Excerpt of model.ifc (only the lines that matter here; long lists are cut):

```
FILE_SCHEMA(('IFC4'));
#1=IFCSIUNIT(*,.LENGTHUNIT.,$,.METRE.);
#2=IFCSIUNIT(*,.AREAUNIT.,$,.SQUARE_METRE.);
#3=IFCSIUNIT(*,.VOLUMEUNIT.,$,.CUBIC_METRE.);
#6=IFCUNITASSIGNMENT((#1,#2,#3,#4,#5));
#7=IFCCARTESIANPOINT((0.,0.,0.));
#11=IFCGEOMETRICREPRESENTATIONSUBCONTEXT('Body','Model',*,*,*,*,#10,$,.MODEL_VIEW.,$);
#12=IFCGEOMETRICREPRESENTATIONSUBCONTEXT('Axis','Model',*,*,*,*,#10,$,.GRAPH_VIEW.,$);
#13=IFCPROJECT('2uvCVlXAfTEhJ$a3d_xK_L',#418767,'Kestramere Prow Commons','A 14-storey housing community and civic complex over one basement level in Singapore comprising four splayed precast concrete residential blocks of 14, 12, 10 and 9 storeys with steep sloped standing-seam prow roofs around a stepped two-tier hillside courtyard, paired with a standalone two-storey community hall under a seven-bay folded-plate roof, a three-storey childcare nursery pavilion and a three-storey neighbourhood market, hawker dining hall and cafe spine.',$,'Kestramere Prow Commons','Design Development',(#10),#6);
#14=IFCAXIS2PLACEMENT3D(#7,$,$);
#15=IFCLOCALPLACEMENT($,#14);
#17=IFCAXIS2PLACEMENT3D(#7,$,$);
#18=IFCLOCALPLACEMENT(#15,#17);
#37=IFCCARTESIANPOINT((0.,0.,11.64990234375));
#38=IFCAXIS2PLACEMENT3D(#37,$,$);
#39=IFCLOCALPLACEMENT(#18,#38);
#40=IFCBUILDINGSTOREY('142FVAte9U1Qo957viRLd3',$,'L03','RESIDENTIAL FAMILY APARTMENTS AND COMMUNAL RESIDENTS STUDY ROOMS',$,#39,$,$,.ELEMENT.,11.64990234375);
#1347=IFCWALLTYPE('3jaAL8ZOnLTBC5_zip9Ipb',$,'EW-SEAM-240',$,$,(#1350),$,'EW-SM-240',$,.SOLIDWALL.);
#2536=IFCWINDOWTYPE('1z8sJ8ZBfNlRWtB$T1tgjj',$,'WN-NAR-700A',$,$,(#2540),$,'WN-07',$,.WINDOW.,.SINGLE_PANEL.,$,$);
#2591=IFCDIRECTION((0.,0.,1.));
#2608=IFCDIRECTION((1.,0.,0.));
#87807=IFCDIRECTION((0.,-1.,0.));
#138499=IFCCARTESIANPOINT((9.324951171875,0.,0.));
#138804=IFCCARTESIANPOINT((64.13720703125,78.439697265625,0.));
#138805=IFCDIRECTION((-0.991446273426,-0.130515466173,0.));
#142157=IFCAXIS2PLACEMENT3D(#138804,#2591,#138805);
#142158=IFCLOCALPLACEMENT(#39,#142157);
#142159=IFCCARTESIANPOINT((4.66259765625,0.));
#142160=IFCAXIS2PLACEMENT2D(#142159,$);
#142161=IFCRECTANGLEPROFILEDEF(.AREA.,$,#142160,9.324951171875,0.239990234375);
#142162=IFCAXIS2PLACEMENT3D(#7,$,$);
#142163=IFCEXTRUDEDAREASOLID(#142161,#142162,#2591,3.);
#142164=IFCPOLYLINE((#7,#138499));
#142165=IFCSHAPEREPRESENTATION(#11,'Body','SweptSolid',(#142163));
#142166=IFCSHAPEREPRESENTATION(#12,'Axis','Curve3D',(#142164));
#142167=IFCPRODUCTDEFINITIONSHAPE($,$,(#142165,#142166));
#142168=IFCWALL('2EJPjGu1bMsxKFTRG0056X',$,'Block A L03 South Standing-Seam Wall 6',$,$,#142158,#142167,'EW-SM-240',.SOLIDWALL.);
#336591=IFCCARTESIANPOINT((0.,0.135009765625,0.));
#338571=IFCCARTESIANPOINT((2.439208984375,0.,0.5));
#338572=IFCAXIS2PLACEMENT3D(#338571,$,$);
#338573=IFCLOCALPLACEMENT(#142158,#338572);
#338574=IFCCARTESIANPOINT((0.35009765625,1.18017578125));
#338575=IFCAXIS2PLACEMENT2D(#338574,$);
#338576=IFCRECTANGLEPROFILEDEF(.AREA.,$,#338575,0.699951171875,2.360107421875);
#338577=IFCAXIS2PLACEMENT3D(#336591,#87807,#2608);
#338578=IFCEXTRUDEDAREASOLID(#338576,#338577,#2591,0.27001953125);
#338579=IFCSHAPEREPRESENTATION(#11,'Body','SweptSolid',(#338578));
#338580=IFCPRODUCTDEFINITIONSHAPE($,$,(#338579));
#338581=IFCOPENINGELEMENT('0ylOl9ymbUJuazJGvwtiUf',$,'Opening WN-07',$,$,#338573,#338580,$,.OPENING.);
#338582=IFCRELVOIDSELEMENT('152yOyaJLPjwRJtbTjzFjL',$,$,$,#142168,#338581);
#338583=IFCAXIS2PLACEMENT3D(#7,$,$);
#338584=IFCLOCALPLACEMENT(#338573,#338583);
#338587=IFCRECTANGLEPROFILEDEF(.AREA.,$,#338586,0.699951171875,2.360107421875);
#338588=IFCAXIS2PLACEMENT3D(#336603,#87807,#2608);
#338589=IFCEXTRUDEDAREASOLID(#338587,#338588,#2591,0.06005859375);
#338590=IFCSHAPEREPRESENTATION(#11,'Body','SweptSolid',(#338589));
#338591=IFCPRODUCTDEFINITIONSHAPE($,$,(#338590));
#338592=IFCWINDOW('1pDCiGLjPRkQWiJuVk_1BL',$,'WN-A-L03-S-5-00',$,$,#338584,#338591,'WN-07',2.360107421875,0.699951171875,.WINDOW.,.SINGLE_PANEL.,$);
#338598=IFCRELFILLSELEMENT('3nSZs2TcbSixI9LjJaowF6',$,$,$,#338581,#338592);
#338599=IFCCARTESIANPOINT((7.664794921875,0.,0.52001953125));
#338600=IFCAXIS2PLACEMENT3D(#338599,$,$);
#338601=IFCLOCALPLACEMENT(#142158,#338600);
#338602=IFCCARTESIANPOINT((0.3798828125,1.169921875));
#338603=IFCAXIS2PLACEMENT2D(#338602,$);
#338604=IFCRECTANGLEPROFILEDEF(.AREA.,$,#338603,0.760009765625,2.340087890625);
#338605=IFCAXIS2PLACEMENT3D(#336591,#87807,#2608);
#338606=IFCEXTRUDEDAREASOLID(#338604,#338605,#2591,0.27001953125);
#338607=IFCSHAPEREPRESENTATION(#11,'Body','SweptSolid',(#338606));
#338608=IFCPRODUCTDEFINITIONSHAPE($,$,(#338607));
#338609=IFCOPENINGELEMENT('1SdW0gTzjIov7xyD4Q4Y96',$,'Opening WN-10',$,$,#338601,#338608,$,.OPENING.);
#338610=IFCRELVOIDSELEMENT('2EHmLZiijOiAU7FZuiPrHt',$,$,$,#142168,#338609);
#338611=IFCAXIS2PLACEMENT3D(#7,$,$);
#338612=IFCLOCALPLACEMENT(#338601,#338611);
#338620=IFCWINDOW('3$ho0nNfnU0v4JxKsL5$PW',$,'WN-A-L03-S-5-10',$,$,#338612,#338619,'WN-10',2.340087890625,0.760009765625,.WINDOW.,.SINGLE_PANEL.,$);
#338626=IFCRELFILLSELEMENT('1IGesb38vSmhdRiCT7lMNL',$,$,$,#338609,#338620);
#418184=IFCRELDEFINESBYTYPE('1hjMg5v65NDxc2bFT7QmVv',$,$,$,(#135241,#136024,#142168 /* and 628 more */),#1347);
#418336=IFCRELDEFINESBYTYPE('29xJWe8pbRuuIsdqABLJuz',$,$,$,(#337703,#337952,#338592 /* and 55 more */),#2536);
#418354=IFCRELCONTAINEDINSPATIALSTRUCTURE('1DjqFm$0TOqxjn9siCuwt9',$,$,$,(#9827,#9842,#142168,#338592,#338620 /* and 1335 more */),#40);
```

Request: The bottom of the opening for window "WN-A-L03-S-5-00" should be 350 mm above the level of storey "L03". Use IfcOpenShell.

```python
import numpy as np
import ifcopenshell
import ifcopenshell.api.geometry
import ifcopenshell.geom
import ifcopenshell.util.element
import ifcopenshell.util.placement
import ifcopenshell.util.shape
import ifcopenshell.util.unit

model = ifcopenshell.open("model.ifc")
unit_scale = ifcopenshell.util.unit.calculate_unit_scale(model)

window = model.by_guid("1pDCiGLjPRkQWiJuVk_1BL")
opening = window.FillsVoids[0].RelatingOpeningElement
storey = ifcopenshell.util.element.get_container(window, ifc_class="IfcBuildingStorey")
level = ifcopenshell.util.placement.get_local_placement(storey.ObjectPlacement)[2, 3]

# The opening's origin need not be at the sill, so measure its lowest point.
shape = ifcopenshell.geom.create_shape(ifcopenshell.geom.settings(), opening)
bottom = ifcopenshell.util.shape.get_shape_bottom_elevation(shape, shape.geometry) / unit_scale
dz = level + 0.35 - bottom

shift = np.array([0.0, 0.0, dz])
# The window is placed relative to its opening, so it follows when the opening moves.
matrix = ifcopenshell.util.placement.get_local_placement(opening.ObjectPlacement)
matrix[:3, 3] += shift
ifcopenshell.api.geometry.edit_object_placement(
    model, product=opening, matrix=matrix, is_si=False, should_transform_children=True
)

print(f"moved by {dz * unit_scale:+.3f} m")

model.write("model_rev.ifc")
```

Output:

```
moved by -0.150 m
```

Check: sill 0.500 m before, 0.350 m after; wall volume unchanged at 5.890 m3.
